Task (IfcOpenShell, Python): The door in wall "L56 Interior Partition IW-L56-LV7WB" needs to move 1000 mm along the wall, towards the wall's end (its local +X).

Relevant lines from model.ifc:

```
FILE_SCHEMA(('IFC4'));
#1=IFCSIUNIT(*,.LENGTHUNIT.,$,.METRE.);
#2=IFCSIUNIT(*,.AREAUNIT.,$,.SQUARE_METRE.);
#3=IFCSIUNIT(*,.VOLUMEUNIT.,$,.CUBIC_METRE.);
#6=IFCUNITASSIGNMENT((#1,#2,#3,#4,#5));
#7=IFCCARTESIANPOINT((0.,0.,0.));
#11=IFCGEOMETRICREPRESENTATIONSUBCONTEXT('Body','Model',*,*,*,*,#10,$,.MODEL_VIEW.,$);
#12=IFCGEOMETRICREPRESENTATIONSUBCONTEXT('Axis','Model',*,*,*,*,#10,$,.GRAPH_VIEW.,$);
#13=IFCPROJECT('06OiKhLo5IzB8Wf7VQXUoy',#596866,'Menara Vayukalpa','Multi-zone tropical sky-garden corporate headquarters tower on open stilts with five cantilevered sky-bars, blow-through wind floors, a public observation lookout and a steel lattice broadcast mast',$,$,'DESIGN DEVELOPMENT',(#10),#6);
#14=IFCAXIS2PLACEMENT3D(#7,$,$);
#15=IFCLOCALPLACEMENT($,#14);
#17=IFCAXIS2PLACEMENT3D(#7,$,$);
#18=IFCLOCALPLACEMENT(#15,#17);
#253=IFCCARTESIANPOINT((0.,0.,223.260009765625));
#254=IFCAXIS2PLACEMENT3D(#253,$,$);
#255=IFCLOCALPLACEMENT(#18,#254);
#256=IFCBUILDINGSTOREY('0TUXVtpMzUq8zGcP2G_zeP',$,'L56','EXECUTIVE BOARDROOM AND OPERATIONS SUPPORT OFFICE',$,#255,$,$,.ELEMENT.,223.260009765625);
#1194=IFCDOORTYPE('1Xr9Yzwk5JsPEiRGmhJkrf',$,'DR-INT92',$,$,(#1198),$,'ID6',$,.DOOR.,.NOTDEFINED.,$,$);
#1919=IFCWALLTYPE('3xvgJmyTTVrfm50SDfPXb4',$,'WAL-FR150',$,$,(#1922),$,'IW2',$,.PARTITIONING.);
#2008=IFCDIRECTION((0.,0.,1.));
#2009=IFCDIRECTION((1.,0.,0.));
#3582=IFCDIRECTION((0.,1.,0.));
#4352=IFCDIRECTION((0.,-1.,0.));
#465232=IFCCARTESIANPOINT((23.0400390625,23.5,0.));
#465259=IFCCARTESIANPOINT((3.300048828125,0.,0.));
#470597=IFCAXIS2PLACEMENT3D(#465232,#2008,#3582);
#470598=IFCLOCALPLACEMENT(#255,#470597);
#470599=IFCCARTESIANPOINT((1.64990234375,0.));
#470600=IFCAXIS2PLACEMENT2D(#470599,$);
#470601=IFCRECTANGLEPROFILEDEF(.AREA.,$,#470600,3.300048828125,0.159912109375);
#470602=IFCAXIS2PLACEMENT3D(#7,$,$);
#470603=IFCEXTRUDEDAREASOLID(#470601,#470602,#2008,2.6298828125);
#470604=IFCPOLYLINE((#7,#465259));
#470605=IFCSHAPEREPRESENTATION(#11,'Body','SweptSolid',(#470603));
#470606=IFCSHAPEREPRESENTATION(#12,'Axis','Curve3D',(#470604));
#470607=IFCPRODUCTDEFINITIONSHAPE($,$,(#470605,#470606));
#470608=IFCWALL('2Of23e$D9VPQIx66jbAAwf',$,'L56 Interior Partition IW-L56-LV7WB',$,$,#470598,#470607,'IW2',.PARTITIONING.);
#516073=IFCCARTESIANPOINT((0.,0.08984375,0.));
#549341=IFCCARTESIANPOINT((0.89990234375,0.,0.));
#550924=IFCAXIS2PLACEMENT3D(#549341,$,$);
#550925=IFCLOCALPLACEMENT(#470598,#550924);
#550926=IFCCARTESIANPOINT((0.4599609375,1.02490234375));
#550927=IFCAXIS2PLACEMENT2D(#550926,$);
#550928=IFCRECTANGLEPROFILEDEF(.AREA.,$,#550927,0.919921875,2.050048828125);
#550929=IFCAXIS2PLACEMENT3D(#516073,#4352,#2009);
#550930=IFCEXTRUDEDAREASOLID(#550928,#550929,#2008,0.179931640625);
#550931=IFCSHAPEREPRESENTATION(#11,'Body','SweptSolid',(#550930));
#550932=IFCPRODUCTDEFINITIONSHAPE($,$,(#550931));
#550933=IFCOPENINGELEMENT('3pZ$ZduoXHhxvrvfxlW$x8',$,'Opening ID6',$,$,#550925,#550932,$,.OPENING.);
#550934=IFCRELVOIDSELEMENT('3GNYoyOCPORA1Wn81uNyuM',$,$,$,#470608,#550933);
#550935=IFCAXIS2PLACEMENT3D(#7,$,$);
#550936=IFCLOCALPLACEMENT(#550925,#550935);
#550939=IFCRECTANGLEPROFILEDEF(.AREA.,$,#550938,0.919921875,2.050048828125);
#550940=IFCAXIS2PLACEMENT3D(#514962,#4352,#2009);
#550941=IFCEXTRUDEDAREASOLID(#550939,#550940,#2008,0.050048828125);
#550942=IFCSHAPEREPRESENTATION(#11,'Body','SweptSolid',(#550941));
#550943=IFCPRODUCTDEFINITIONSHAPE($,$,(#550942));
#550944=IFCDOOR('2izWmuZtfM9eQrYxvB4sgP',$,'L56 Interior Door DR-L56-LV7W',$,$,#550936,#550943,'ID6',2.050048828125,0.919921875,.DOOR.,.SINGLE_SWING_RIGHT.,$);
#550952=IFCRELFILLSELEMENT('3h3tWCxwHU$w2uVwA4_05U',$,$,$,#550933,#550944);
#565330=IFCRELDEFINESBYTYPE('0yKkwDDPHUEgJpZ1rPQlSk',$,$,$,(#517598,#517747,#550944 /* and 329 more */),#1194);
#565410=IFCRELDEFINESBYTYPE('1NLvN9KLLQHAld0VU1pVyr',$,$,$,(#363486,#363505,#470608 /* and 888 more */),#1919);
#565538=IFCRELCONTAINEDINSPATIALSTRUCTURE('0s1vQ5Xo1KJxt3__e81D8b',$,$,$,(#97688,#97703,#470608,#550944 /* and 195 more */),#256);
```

```python
import ifcopenshell
import ifcopenshell.api.geometry
import ifcopenshell.util.placement
import ifcopenshell.util.unit

model = ifcopenshell.open("model.ifc")
unit_scale = ifcopenshell.util.unit.calculate_unit_scale(model)

door = model.by_guid("2izWmuZtfM9eQrYxvB4sgP")
opening = door.FillsVoids[0].RelatingOpeningElement
wall = opening.VoidsElements[0].RelatingBuildingElement

wall_matrix = ifcopenshell.util.placement.get_local_placement(wall.ObjectPlacement)
shift = wall_matrix[:3, 0] * 1 / unit_scale
before = ifcopenshell.util.placement.get_local_placement(door.ObjectPlacement)[:3, 3].copy()

# The door is placed relative to its opening, so it follows when the opening moves.
matrix = ifcopenshell.util.placement.get_local_placement(opening.ObjectPlacement)
matrix[:3, 3] += shift
ifcopenshell.api.geometry.edit_object_placement(
    model, product=opening, matrix=matrix, is_si=False, should_transform_children=True
)

after = ifcopenshell.util.placement.get_local_placement(door.ObjectPlacement)[:3, 3]
print("door moved by", (after - before).round(3) + 0.0)

model.write("model_edited.ifc")
```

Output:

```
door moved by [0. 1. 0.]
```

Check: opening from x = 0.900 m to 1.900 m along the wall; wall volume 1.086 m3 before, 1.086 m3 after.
